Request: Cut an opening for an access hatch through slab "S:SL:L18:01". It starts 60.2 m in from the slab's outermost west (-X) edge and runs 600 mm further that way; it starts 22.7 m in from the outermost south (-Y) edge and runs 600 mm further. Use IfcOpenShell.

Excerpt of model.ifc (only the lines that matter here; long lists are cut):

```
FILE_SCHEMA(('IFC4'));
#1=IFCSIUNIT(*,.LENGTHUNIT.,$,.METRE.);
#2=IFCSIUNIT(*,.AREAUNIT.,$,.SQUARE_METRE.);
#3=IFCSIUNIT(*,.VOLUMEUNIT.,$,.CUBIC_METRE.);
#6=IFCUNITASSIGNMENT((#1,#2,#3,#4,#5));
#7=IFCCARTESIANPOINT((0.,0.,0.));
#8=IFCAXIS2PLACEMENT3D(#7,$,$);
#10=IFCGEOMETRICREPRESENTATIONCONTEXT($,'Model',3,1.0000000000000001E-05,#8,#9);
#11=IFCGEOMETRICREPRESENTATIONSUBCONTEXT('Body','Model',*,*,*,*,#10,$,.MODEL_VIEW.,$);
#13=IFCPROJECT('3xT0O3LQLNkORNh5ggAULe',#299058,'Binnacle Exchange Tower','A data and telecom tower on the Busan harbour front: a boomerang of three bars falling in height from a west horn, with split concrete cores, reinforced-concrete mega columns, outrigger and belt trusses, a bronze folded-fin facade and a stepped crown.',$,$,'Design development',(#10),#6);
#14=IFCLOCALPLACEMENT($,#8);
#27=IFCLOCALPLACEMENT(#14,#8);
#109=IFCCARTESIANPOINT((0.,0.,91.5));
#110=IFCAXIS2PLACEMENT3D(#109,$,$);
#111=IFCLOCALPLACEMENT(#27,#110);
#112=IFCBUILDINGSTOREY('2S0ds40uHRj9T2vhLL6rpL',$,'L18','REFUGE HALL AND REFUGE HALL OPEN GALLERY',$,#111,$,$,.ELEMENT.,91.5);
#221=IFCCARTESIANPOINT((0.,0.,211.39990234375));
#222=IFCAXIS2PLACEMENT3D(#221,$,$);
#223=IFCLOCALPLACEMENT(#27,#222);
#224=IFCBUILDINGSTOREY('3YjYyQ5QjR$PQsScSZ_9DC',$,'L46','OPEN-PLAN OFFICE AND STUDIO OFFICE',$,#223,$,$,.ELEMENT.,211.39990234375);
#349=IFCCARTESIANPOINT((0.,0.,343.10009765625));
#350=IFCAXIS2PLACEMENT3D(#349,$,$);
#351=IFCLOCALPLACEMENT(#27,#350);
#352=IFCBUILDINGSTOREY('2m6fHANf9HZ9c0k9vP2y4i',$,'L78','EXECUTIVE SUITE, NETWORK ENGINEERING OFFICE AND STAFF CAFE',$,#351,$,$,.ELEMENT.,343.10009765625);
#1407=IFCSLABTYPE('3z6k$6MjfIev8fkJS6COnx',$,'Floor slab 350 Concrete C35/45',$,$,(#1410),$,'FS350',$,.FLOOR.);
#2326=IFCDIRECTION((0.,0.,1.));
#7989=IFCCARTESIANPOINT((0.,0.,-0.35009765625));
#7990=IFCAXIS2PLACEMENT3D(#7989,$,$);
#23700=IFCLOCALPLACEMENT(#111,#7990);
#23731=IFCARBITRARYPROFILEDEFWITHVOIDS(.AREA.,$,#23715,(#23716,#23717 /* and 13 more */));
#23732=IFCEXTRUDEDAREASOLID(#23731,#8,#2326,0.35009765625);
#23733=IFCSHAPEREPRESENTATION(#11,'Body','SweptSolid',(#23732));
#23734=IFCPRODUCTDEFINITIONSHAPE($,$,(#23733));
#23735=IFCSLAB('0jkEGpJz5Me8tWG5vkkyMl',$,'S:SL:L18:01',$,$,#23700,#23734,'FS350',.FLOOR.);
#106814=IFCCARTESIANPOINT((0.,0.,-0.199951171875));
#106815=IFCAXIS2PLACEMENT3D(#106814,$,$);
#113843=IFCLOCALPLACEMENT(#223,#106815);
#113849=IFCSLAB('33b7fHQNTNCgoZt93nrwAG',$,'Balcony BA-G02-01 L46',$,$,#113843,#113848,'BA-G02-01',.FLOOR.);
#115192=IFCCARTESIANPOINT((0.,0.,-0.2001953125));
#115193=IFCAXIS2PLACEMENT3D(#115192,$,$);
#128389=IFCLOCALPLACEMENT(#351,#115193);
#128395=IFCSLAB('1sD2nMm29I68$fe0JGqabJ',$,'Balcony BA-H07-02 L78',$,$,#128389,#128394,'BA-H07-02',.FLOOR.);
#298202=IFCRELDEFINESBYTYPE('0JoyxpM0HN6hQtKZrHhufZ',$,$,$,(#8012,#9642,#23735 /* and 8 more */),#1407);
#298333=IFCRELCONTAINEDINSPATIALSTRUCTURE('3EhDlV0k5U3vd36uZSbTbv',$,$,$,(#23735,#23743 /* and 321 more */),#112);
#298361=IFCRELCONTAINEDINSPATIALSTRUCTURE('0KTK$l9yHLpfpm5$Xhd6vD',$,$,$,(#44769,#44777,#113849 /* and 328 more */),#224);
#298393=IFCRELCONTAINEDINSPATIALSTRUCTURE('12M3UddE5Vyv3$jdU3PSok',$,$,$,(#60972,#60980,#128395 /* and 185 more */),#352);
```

```python
import numpy as np
import ifcopenshell
import ifcopenshell.api.feature
import ifcopenshell.api.geometry
import ifcopenshell.api.root
import ifcopenshell.geom
import ifcopenshell.util.placement
import ifcopenshell.util.representation
import ifcopenshell.util.shape
import ifcopenshell.util.unit

model = ifcopenshell.open("model.ifc")
unit_scale = ifcopenshell.util.unit.calculate_unit_scale(model)
settings = ifcopenshell.geom.settings()


def volume(element):
    """Net volume in cubic metres, openings subtracted."""
    shape = ifcopenshell.geom.create_shape(settings, element)
    return ifcopenshell.util.shape.get_volume(shape.geometry)


slab = model.by_id(23735)
before = volume(slab)

# Extent in the slab's own axes, in metres. The edges named are its -X and -Y sides.
slab_shape = ifcopenshell.geom.create_shape(settings, slab)
vertices = ifcopenshell.util.shape.get_vertices(slab_shape.geometry)
x_min, y_min, bottom = vertices.min(axis=0)
top = vertices[:, 2].max()

opening = ifcopenshell.api.root.create_entity(model, ifc_class="IfcOpeningElement", name="Access hatch opening", predefined_type="OPENING")
context = ifcopenshell.util.representation.get_context(model, "Model", "Body", "MODEL_VIEW")
width, depth = 0.6, 0.6
outline = [(0.0, 0.0), (width, 0.0), (width, depth), (0.0, depth), (0.0, 0.0)]
# Overshoot both faces by 50 mm so the cut is clean.
shape = ifcopenshell.api.geometry.add_slab_representation(
    model, context=context, depth=top - bottom + 0.1, polyline=outline
)
ifcopenshell.api.geometry.assign_representation(model, product=opening, representation=shape)

matrix = ifcopenshell.util.placement.get_local_placement(slab.ObjectPlacement)
matrix[:, 3] = matrix @ np.append(np.array([x_min + 60.2, y_min + 22.7, bottom - 0.05]) / unit_scale, 1.0)
ifcopenshell.api.geometry.edit_object_placement(model, product=opening, matrix=matrix, is_si=False)
ifcopenshell.api.feature.add_feature(model, feature=opening, element=slab)

after = volume(slab)

print(f"slab volume {before:.3f} -> {after:.3f} m3")

model.write("model-out.ifc")
```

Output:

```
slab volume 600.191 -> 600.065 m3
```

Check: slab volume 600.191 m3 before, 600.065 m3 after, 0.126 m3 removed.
